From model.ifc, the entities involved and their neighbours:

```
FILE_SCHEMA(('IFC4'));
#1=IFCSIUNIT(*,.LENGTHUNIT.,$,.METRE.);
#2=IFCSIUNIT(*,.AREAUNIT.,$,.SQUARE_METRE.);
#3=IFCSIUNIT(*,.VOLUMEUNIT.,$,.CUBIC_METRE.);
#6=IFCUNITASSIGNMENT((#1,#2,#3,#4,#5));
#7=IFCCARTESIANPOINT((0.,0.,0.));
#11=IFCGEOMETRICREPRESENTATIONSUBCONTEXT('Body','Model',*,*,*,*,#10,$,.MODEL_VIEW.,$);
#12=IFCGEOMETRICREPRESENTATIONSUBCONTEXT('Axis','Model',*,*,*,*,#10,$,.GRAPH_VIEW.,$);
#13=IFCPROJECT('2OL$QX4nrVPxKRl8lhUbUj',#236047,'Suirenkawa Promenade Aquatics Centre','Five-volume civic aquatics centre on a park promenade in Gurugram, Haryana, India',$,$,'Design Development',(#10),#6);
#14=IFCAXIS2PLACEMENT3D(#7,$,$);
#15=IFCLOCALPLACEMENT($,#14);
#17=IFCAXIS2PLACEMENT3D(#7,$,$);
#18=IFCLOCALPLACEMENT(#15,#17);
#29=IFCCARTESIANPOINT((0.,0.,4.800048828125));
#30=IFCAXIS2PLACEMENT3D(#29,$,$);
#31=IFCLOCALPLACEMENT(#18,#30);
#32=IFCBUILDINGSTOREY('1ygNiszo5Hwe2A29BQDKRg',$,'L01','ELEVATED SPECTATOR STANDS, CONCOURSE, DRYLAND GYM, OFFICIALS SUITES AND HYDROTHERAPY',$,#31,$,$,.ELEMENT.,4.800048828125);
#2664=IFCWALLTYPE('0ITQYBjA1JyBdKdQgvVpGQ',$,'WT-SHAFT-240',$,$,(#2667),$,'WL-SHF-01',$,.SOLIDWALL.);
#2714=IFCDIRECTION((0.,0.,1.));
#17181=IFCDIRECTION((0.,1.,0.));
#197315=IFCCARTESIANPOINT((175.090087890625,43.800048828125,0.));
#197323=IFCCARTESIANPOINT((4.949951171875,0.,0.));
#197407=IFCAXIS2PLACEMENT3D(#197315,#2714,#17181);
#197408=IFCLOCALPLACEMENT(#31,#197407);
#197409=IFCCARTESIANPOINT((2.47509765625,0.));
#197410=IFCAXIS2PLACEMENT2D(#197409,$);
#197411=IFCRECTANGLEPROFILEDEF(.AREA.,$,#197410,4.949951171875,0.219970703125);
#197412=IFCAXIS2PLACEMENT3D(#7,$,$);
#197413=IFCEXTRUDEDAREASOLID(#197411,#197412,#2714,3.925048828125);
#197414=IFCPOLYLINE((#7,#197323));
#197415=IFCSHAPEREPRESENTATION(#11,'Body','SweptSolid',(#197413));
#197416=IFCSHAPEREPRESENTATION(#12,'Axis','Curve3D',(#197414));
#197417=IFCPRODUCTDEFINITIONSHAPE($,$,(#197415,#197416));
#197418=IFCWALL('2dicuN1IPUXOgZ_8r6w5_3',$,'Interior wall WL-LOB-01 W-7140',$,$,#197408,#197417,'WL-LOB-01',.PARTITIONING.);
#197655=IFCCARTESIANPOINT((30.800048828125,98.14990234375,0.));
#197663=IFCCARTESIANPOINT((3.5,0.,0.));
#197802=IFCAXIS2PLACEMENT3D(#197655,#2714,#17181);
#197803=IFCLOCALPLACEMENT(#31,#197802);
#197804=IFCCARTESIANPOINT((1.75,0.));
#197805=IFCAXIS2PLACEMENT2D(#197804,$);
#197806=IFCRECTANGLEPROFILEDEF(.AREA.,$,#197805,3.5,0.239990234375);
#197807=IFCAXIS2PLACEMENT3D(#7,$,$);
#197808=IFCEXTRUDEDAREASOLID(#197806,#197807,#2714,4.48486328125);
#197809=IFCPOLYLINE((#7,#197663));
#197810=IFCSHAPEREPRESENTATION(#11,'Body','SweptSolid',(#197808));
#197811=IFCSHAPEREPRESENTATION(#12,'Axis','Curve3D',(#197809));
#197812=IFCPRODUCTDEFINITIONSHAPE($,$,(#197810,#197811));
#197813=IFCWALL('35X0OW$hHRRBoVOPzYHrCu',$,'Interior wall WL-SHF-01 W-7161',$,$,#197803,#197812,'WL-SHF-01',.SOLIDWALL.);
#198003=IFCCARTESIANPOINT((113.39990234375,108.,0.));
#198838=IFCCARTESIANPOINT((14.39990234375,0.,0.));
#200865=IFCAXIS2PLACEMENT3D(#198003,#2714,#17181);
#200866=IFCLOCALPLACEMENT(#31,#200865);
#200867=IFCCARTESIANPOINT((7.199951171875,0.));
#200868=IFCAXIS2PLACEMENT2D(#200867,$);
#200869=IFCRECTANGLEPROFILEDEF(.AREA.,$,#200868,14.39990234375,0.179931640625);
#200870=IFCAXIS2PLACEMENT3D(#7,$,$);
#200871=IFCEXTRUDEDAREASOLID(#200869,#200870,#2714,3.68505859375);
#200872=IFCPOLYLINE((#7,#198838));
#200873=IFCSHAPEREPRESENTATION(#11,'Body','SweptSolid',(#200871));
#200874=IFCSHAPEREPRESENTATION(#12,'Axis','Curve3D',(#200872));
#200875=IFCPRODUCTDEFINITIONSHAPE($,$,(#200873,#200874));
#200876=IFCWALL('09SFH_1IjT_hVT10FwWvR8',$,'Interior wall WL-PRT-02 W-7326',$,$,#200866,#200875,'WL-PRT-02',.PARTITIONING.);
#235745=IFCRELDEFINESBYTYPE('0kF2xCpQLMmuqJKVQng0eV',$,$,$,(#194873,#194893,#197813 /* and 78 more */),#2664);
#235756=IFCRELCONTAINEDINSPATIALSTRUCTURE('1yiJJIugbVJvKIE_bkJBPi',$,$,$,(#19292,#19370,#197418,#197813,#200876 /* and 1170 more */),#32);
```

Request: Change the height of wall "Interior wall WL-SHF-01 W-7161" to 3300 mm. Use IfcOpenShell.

```python
import ifcopenshell
import ifcopenshell.geom
import ifcopenshell.util.representation
import ifcopenshell.util.shape

model = ifcopenshell.open("model.ifc")
settings = ifcopenshell.geom.settings()


def volume(element):
    """Net volume in cubic metres, openings subtracted."""
    shape = ifcopenshell.geom.create_shape(settings, element)
    return ifcopenshell.util.shape.get_volume(shape.geometry)


wall = model.by_id(197813)
before = volume(wall)

body = ifcopenshell.util.representation.get_representation(wall, "Model", "Body")
solid = body.Items[0]
old_height = solid.Depth
solid.Depth = 3.3
after = volume(wall)

print(f"height {old_height:g} -> {solid.Depth:g}, volume {before:.3f} -> {after:.3f} m3")

model.write("model_v2.ifc")
```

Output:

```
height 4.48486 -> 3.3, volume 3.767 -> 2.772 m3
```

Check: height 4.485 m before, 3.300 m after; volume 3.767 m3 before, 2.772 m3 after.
